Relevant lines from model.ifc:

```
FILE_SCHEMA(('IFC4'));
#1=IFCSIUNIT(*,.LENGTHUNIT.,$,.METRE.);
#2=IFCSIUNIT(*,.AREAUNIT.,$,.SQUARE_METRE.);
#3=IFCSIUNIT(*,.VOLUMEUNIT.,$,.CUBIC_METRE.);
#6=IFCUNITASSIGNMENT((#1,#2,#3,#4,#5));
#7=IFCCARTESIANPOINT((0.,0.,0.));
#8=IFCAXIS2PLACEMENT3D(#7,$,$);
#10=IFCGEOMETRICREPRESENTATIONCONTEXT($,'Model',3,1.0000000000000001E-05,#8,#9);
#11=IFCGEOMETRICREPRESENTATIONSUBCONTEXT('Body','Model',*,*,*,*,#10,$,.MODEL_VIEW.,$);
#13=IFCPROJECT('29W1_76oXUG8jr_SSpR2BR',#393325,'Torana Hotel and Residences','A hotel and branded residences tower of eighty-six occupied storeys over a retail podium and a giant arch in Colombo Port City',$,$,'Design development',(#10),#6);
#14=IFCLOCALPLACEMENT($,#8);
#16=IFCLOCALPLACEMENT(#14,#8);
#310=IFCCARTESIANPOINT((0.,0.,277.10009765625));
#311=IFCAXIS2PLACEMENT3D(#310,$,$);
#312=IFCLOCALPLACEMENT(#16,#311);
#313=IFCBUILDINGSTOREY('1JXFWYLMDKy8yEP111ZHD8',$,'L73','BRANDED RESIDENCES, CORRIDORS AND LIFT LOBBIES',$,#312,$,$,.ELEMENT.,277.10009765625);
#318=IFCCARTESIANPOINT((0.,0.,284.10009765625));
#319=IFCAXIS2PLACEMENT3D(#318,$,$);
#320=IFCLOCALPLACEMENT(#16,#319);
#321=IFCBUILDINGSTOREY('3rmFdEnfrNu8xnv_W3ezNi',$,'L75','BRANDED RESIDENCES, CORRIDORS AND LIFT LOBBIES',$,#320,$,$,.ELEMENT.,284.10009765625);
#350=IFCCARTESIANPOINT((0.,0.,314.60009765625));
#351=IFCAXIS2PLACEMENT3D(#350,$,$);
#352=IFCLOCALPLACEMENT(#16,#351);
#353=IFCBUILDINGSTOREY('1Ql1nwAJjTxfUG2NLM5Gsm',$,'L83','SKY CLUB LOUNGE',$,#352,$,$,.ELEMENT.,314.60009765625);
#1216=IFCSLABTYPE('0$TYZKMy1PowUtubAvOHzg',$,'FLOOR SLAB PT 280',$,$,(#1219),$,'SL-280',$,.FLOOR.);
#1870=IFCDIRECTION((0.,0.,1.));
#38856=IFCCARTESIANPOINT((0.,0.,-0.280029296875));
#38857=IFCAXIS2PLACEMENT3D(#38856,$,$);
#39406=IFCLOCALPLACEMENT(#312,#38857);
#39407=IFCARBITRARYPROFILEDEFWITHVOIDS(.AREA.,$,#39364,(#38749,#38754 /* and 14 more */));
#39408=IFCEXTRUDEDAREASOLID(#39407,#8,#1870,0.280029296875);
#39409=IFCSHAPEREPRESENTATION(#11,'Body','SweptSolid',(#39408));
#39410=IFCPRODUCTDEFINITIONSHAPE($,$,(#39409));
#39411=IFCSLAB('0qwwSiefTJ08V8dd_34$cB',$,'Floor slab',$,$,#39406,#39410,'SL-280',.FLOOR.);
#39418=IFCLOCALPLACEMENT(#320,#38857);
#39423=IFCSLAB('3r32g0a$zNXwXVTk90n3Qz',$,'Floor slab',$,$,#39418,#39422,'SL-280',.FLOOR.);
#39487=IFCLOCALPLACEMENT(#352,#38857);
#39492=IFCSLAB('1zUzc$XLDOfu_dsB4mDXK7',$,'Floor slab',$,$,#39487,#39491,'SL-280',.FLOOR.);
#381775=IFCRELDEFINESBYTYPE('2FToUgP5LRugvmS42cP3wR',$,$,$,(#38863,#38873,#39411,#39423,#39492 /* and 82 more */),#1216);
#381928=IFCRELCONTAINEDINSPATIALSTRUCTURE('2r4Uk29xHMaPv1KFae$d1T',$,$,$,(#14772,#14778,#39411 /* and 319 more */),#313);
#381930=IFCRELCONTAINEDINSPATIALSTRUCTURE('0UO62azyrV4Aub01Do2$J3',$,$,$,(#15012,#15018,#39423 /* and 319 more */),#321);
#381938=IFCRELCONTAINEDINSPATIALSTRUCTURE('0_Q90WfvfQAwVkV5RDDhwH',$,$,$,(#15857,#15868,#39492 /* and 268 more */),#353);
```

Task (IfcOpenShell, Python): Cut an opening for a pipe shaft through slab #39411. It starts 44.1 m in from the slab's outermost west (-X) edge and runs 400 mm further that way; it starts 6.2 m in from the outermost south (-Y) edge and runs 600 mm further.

```python
import numpy as np
import ifcopenshell
import ifcopenshell.api.feature
import ifcopenshell.api.geometry
import ifcopenshell.api.root
import ifcopenshell.geom
import ifcopenshell.util.placement
import ifcopenshell.util.representation
import ifcopenshell.util.shape
import ifcopenshell.util.unit

model = ifcopenshell.open("model.ifc")
unit_scale = ifcopenshell.util.unit.calculate_unit_scale(model)
settings = ifcopenshell.geom.settings()


def volume(element):
    """Net volume in cubic metres, openings subtracted."""
    shape = ifcopenshell.geom.create_shape(settings, element)
    return ifcopenshell.util.shape.get_volume(shape.geometry)


slab = model.by_id(39411)
before = volume(slab)

# Extent in the slab's own axes, in metres. The edges named are its -X and -Y sides.
slab_shape = ifcopenshell.geom.create_shape(settings, slab)
vertices = ifcopenshell.util.shape.get_vertices(slab_shape.geometry)
x_min, y_min, bottom = vertices.min(axis=0)
top = vertices[:, 2].max()

opening = ifcopenshell.api.root.create_entity(model, ifc_class="IfcOpeningElement", name="Pipe shaft opening", predefined_type="OPENING")
context = ifcopenshell.util.representation.get_context(model, "Model", "Body", "MODEL_VIEW")
width, depth = 0.4, 0.6
outline = [(0.0, 0.0), (width, 0.0), (width, depth), (0.0, depth), (0.0, 0.0)]
# Overshoot both faces by 50 mm so the cut is clean.
shape = ifcopenshell.api.geometry.add_slab_representation(
    model, context=context, depth=top - bottom + 0.1, polyline=outline
)
ifcopenshell.api.geometry.assign_representation(model, product=opening, representation=shape)

matrix = ifcopenshell.util.placement.get_local_placement(slab.ObjectPlacement)
matrix[:, 3] = matrix @ np.append(np.array([x_min + 44.1, y_min + 6.2, bottom - 0.05]) / unit_scale, 1.0)
ifcopenshell.api.geometry.edit_object_placement(model, product=opening, matrix=matrix, is_si=False)
ifcopenshell.api.feature.add_feature(model, feature=opening, element=slab)

after = volume(slab)

print(f"slab volume {before:.3f} -> {after:.3f} m3")

model.write("model_updated.ifc")
```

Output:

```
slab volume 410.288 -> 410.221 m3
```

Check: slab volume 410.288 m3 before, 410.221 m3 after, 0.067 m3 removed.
